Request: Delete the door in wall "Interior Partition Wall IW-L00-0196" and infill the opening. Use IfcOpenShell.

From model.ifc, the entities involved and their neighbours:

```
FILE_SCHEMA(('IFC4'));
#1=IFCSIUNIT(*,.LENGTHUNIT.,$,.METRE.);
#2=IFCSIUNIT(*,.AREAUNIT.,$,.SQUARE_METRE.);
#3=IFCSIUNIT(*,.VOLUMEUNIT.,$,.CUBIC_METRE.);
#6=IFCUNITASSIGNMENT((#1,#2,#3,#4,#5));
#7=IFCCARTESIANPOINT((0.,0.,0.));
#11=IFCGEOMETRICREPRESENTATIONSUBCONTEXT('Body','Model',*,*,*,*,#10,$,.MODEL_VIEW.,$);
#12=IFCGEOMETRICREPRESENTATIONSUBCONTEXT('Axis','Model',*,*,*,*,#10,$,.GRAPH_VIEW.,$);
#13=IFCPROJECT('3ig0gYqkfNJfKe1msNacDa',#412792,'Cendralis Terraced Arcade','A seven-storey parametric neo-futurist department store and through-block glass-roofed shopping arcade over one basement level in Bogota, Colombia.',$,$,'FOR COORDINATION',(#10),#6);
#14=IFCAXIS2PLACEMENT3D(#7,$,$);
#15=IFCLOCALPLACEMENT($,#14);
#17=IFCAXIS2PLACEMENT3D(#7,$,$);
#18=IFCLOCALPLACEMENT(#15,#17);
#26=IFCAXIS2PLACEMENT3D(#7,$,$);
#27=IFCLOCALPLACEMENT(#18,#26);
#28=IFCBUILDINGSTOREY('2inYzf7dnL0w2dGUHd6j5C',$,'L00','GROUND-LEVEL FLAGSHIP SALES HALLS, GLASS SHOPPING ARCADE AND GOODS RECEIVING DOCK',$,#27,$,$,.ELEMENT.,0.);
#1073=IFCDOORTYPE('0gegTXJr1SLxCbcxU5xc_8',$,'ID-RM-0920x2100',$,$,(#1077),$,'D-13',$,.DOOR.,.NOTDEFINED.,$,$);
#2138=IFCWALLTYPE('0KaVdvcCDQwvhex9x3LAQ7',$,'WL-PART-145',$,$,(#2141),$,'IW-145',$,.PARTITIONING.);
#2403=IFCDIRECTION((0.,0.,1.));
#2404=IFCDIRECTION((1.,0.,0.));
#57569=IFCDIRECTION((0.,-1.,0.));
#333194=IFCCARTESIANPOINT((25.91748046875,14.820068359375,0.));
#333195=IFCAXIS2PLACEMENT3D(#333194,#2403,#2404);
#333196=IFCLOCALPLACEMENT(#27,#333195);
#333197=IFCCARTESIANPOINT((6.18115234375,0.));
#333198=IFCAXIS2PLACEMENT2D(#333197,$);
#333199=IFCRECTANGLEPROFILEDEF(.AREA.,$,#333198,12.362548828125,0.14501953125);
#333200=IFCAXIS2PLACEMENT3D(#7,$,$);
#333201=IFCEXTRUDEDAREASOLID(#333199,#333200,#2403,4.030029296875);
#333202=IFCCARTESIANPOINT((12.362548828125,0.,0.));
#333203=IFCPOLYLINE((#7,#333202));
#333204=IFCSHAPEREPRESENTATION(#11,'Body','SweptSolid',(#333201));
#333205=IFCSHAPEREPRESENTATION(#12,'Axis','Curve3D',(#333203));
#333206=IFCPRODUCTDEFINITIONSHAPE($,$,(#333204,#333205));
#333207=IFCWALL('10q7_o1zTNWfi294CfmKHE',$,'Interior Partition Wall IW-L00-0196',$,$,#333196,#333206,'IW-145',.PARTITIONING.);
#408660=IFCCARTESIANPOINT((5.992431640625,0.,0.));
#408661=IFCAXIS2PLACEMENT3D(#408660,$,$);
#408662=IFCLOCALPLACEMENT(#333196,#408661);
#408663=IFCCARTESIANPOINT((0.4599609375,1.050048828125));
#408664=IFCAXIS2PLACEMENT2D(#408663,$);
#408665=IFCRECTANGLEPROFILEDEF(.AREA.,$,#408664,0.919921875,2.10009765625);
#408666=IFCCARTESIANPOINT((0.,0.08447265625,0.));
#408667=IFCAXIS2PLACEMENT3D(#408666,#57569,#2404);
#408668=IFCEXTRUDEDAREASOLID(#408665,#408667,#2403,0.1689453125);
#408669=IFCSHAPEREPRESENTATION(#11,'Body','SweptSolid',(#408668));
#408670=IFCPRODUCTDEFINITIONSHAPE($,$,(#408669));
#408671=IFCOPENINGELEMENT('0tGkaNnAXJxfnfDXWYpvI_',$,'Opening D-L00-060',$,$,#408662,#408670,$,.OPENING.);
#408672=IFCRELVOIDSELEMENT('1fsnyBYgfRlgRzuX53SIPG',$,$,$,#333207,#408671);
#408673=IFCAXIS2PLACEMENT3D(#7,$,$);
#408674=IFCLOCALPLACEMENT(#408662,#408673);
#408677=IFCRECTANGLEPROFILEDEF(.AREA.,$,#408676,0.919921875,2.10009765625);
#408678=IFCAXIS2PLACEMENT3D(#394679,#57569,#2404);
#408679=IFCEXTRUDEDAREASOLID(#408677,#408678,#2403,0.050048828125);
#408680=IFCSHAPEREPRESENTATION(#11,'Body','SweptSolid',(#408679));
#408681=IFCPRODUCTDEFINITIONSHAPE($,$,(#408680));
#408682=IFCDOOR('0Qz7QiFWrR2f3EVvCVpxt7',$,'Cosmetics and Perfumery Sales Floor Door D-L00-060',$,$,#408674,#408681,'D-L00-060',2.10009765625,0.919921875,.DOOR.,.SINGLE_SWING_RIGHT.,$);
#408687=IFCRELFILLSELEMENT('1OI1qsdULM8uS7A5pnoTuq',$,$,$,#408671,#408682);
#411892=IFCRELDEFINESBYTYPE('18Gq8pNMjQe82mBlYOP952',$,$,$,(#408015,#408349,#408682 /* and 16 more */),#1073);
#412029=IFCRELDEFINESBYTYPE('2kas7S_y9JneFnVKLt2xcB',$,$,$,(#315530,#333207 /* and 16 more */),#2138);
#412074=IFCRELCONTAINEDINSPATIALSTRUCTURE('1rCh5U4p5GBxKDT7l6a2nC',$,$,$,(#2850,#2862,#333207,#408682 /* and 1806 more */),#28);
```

```python
import ifcopenshell
import ifcopenshell.api.feature
import ifcopenshell.api.root
import ifcopenshell.geom
import ifcopenshell.util.shape

model = ifcopenshell.open("model.ifc")
settings = ifcopenshell.geom.settings()


def volume(element):
    """Net volume in cubic metres, openings subtracted."""
    shape = ifcopenshell.geom.create_shape(settings, element)
    return ifcopenshell.util.shape.get_volume(shape.geometry)


door = model.by_guid("0Qz7QiFWrR2f3EVvCVpxt7")
opening = door.FillsVoids[0].RelatingOpeningElement
wall = opening.VoidsElements[0].RelatingBuildingElement
before = volume(wall)

ifcopenshell.api.root.remove_product(model, product=door)
ifcopenshell.api.feature.remove_feature(model, feature=opening)

after = volume(wall)

print(f"wall volume {before:.3f} -> {after:.3f} m3")

model.write("model-out.ifc")
```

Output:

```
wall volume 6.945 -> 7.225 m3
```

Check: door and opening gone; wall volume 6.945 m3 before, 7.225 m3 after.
